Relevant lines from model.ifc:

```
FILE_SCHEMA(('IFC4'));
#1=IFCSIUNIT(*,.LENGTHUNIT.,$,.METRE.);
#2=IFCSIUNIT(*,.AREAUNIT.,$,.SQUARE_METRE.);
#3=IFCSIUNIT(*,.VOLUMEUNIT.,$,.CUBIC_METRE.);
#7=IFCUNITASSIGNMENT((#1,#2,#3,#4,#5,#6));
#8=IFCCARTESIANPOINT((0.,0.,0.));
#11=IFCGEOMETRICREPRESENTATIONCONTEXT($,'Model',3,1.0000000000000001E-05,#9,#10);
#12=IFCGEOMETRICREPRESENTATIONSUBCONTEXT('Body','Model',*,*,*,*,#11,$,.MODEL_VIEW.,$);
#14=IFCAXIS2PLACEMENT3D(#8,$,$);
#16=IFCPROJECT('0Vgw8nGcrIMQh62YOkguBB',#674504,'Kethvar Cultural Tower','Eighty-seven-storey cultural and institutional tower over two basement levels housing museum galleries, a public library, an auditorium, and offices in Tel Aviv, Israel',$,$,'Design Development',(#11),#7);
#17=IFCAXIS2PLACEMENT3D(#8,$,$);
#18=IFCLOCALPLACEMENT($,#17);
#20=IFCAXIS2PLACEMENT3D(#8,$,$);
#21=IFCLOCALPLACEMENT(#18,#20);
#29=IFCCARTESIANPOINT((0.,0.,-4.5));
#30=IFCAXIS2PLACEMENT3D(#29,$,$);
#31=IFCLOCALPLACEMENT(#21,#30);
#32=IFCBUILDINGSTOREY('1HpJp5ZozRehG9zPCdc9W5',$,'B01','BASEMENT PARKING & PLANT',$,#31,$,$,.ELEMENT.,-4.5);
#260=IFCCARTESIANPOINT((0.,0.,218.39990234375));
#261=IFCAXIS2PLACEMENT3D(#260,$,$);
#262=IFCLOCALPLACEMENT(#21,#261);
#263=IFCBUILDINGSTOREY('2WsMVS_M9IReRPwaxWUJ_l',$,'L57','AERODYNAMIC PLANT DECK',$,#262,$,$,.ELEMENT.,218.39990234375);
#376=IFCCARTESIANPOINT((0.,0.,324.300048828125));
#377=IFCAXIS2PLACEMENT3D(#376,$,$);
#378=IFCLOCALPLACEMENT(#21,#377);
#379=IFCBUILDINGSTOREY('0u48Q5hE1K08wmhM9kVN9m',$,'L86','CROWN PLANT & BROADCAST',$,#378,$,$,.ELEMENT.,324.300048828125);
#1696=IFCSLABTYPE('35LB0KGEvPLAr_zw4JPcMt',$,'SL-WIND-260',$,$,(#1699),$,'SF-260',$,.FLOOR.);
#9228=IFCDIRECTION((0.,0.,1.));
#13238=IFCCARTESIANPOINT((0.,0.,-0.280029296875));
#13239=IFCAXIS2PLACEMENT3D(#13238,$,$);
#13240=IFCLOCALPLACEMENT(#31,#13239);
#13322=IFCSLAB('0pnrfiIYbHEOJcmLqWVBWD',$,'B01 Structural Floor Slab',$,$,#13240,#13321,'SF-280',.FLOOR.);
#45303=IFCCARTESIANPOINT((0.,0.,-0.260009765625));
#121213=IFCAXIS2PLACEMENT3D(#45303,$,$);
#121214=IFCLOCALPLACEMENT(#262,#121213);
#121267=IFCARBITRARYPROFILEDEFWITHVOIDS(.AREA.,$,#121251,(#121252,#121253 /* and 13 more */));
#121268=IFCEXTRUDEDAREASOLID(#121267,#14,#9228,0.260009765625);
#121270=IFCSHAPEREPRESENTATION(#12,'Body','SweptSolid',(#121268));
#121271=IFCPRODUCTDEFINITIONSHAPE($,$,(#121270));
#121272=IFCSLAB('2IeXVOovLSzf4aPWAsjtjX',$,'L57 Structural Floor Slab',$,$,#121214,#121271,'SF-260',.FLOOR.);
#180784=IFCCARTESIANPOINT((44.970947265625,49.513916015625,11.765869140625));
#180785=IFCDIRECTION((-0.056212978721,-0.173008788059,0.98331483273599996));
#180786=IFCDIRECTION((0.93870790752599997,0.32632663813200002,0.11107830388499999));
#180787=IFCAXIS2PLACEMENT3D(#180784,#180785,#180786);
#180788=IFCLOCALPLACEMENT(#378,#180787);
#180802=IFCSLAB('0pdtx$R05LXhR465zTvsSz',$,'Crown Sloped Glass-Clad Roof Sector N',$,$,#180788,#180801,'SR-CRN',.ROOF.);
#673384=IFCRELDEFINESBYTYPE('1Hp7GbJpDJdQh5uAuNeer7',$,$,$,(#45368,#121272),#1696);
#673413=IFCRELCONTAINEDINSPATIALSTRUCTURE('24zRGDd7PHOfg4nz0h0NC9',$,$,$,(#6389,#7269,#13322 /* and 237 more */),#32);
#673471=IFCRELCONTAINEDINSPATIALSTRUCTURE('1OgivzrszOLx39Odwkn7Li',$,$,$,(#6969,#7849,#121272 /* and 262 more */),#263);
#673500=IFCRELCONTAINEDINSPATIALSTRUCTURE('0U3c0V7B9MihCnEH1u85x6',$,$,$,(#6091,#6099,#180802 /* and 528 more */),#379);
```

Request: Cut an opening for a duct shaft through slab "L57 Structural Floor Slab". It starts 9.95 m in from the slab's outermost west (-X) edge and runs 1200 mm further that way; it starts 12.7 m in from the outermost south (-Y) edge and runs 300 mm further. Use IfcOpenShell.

```python
import numpy as np
import ifcopenshell
import ifcopenshell.api.feature
import ifcopenshell.api.geometry
import ifcopenshell.api.root
import ifcopenshell.geom
import ifcopenshell.util.placement
import ifcopenshell.util.representation
import ifcopenshell.util.shape
import ifcopenshell.util.unit

model = ifcopenshell.open("model.ifc")
unit_scale = ifcopenshell.util.unit.calculate_unit_scale(model)
settings = ifcopenshell.geom.settings()


def volume(element):
    """Net volume in cubic metres, openings subtracted."""
    shape = ifcopenshell.geom.create_shape(settings, element)
    return ifcopenshell.util.shape.get_volume(shape.geometry)


slab = model.by_guid("2IeXVOovLSzf4aPWAsjtjX")
before = volume(slab)

# Extent in the slab's own axes, in metres. The edges named are its -X and -Y sides.
slab_shape = ifcopenshell.geom.create_shape(settings, slab)
vertices = ifcopenshell.util.shape.get_vertices(slab_shape.geometry)
x_min, y_min, bottom = vertices.min(axis=0)
top = vertices[:, 2].max()

opening = ifcopenshell.api.root.create_entity(model, ifc_class="IfcOpeningElement", name="Duct shaft opening", predefined_type="OPENING")
context = ifcopenshell.util.representation.get_context(model, "Model", "Body", "MODEL_VIEW")
width, depth = 1.2, 0.3
outline = [(0.0, 0.0), (width, 0.0), (width, depth), (0.0, depth), (0.0, 0.0)]
# Overshoot both faces by 50 mm so the cut is clean.
shape = ifcopenshell.api.geometry.add_slab_representation(
    model, context=context, depth=top - bottom + 0.1, polyline=outline
)
ifcopenshell.api.geometry.assign_representation(model, product=opening, representation=shape)

matrix = ifcopenshell.util.placement.get_local_placement(slab.ObjectPlacement)
matrix[:, 3] = matrix @ np.append(np.array([x_min + 9.95, y_min + 12.7, bottom - 0.05]) / unit_scale, 1.0)
ifcopenshell.api.geometry.edit_object_placement(model, product=opening, matrix=matrix, is_si=False)
ifcopenshell.api.feature.add_feature(model, feature=opening, element=slab)

after = volume(slab)

print(f"slab volume {before:.3f} -> {after:.3f} m3")

model.write("model_edited.ifc")
```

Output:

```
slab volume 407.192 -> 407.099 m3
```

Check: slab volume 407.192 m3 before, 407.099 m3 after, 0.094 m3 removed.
